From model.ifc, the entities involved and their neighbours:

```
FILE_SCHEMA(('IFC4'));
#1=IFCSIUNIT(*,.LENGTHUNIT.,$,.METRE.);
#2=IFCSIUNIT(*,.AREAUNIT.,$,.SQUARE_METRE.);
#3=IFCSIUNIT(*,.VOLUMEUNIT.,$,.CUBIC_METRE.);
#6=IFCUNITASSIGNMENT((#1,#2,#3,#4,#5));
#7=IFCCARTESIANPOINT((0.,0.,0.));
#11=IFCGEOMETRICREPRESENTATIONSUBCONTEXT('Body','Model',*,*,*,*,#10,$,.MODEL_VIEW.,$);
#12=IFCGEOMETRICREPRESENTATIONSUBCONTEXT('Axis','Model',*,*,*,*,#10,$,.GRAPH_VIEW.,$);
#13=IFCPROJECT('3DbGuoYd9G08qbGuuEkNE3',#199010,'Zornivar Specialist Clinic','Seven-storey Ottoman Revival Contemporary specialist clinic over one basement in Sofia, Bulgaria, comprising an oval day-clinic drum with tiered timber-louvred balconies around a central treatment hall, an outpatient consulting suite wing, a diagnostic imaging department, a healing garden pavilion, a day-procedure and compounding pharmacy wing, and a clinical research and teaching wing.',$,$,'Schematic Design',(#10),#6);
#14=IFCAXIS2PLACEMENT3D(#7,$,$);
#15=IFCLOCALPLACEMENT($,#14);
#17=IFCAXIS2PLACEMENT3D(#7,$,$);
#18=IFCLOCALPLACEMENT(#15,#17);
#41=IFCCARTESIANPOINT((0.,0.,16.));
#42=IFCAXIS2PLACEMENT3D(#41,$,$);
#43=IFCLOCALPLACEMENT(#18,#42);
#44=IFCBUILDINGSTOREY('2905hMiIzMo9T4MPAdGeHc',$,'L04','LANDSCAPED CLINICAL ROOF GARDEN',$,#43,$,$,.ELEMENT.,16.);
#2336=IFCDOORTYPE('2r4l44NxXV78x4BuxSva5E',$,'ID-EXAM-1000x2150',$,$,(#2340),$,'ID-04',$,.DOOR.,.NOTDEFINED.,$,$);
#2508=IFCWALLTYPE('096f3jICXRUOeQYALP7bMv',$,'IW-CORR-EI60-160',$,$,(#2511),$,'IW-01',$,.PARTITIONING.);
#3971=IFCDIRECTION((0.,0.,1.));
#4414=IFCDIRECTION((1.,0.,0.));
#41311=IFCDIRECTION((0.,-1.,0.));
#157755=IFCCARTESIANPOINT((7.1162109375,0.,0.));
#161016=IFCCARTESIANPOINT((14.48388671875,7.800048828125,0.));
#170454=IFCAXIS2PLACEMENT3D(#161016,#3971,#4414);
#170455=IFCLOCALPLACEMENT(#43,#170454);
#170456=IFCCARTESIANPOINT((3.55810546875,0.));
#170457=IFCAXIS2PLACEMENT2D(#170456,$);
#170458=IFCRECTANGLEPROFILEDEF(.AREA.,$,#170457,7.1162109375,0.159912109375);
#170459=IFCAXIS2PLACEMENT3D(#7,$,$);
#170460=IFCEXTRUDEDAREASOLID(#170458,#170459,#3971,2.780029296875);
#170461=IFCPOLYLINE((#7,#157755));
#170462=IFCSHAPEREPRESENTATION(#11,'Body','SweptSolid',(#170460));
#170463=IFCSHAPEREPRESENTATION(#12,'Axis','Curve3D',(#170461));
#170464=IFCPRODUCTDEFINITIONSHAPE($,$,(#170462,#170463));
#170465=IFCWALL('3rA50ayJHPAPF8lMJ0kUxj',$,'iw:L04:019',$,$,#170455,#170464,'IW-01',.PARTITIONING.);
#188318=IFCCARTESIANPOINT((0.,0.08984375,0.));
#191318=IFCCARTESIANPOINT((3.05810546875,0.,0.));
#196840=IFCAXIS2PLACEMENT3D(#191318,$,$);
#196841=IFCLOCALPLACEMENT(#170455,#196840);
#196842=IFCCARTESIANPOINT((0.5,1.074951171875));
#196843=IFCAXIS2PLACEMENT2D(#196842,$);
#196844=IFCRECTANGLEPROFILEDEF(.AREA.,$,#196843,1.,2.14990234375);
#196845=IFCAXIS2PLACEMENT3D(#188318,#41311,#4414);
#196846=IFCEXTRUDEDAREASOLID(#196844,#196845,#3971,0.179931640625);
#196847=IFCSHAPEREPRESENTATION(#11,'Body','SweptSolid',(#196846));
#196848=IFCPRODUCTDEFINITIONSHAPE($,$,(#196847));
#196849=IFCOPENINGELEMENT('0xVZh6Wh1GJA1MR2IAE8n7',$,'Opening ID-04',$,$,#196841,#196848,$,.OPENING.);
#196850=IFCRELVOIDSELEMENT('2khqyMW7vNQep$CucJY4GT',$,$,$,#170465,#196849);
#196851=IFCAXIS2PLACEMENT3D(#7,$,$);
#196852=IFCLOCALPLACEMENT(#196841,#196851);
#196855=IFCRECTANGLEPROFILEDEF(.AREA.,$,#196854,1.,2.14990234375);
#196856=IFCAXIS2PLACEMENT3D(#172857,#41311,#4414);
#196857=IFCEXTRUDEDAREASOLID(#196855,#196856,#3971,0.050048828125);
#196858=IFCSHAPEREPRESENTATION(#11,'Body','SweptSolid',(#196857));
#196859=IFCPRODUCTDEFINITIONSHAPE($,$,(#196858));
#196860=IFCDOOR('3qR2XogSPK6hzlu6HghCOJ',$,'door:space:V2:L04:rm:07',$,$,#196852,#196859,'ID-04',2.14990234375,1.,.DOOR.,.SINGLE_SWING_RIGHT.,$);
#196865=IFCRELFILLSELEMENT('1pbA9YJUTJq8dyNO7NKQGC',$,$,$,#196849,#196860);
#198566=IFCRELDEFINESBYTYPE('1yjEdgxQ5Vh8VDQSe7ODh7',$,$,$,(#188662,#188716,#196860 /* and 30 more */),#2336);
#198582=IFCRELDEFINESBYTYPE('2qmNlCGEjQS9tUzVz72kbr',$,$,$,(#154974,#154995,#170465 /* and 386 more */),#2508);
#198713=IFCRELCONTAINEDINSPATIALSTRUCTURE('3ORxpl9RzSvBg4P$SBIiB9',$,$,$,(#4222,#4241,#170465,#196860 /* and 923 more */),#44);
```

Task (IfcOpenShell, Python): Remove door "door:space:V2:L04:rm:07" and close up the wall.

```python
import ifcopenshell
import ifcopenshell.api.feature
import ifcopenshell.api.root
import ifcopenshell.geom
import ifcopenshell.util.shape

model = ifcopenshell.open("model.ifc")
settings = ifcopenshell.geom.settings()


def volume(element):
    """Net volume in cubic metres, openings subtracted."""
    shape = ifcopenshell.geom.create_shape(settings, element)
    return ifcopenshell.util.shape.get_volume(shape.geometry)


door = model.by_guid("3qR2XogSPK6hzlu6HghCOJ")
opening = door.FillsVoids[0].RelatingOpeningElement
wall = opening.VoidsElements[0].RelatingBuildingElement
before = volume(wall)

ifcopenshell.api.root.remove_product(model, product=door)
ifcopenshell.api.feature.remove_feature(model, feature=opening)

after = volume(wall)

print(f"wall volume {before:.3f} -> {after:.3f} m3")

model.write("model_v2.ifc")
```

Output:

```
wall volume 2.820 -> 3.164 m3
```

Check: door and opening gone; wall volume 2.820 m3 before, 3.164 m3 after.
